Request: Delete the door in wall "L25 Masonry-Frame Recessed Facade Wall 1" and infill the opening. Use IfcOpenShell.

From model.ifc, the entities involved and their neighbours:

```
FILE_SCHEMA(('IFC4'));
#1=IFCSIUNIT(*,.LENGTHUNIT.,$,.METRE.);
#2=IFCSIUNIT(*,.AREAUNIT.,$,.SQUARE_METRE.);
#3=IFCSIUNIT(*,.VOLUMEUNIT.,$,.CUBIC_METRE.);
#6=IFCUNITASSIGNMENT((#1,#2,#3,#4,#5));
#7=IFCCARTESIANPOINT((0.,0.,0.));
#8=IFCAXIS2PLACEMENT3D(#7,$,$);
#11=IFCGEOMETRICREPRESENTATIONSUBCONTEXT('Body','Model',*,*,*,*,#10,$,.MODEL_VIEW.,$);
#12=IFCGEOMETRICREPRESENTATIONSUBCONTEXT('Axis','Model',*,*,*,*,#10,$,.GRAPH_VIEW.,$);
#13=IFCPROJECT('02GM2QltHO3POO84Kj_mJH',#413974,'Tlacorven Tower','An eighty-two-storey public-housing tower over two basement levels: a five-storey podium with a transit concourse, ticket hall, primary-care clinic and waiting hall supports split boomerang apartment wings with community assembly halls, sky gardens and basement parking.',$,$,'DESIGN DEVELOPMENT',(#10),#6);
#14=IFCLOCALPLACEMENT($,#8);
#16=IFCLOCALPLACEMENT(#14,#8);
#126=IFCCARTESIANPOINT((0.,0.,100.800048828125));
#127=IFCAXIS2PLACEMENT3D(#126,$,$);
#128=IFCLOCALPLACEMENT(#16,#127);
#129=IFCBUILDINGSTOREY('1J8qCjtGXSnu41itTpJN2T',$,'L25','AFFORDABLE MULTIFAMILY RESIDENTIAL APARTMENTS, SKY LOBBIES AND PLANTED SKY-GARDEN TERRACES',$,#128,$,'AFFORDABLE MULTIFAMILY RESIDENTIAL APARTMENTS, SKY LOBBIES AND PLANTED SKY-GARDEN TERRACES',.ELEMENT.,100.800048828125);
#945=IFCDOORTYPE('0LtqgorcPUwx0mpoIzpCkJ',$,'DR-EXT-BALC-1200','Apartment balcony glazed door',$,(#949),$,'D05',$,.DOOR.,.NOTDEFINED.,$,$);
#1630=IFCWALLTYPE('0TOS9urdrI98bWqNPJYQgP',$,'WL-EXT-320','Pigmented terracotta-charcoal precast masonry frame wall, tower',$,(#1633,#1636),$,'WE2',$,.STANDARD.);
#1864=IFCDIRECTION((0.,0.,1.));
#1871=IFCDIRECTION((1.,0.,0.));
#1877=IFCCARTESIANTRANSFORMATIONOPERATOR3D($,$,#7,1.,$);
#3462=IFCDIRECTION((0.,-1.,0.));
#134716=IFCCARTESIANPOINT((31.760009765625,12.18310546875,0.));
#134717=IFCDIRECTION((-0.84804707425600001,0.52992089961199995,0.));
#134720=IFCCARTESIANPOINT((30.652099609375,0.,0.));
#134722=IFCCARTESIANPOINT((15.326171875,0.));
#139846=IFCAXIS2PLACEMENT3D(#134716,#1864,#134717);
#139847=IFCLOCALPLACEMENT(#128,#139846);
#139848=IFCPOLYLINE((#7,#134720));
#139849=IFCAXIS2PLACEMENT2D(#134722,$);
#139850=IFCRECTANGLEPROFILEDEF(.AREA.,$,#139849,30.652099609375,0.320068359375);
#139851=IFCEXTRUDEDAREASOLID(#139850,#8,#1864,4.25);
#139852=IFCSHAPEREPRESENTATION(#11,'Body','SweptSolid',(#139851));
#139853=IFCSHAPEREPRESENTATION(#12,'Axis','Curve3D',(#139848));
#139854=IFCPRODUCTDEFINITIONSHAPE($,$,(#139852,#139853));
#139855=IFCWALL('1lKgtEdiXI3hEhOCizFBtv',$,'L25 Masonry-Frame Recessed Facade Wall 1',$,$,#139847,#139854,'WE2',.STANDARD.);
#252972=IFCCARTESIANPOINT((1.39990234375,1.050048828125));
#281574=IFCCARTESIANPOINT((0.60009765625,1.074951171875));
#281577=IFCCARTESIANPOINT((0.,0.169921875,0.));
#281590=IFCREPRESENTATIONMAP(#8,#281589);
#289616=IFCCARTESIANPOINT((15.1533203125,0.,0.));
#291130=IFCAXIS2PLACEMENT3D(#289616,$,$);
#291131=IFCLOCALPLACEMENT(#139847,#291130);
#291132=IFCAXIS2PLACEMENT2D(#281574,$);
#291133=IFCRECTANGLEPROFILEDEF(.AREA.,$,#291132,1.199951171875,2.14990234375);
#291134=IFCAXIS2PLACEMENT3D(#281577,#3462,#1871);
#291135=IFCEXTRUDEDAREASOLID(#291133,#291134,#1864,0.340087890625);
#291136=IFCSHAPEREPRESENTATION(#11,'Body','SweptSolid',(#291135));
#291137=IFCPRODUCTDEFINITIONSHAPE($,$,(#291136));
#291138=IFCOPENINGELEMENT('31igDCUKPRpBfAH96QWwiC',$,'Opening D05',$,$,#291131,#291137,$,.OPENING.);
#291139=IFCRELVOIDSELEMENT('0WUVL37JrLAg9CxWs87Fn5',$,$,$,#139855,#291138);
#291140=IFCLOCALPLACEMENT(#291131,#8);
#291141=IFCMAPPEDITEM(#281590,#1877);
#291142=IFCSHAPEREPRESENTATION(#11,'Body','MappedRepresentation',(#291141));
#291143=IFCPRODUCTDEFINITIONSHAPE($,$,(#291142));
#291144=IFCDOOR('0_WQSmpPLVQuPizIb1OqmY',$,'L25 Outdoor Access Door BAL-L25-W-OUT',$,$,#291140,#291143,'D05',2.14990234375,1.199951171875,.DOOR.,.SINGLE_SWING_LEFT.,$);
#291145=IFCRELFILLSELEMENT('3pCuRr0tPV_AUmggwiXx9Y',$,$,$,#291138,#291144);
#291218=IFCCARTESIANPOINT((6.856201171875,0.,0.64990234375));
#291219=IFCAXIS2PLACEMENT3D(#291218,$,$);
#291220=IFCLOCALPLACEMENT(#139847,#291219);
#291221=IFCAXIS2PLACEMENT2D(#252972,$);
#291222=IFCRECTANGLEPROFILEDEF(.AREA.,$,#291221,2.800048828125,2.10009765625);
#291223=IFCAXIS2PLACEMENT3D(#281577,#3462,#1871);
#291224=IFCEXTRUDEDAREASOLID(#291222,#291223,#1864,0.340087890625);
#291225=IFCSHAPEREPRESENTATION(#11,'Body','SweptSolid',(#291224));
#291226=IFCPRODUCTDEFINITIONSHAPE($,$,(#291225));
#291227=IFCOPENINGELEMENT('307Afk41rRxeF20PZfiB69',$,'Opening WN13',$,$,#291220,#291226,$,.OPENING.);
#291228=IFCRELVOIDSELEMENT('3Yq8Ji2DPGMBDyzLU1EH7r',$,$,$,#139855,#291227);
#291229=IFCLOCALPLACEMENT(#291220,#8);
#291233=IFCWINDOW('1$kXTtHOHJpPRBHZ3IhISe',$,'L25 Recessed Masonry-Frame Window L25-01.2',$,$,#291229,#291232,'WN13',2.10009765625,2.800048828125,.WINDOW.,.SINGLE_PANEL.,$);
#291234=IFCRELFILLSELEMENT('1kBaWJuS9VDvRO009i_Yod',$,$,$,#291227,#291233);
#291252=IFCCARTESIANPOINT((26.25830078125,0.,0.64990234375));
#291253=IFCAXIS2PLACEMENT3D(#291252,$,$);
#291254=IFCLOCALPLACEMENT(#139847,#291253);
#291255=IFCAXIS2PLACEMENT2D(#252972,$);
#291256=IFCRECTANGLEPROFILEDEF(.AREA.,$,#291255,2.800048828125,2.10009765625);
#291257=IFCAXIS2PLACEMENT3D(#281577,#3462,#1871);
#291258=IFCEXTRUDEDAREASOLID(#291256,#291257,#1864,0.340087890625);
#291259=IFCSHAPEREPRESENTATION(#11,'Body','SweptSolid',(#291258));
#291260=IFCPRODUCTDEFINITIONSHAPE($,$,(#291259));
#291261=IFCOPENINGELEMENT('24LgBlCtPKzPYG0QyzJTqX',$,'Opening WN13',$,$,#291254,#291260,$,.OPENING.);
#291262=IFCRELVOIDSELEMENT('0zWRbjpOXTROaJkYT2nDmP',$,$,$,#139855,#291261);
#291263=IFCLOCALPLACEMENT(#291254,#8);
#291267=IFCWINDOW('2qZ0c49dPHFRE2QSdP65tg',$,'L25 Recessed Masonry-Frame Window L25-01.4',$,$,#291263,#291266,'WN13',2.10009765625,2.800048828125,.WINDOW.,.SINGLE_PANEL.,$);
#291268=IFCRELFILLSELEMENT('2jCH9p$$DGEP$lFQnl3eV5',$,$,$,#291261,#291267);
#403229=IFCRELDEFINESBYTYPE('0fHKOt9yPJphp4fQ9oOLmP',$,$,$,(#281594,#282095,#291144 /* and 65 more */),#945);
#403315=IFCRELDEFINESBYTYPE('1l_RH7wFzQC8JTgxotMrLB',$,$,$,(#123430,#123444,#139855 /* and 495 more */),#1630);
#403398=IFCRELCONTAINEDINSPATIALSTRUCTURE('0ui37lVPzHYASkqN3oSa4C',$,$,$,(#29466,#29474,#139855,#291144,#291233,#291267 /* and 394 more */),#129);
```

```python
import ifcopenshell
import ifcopenshell.api.feature
import ifcopenshell.api.root
import ifcopenshell.geom
import ifcopenshell.util.shape

model = ifcopenshell.open("model.ifc")
settings = ifcopenshell.geom.settings()


def volume(element):
    """Net volume in cubic metres, openings subtracted."""
    shape = ifcopenshell.geom.create_shape(settings, element)
    return ifcopenshell.util.shape.get_volume(shape.geometry)


door = model.by_id(291144)
opening = door.FillsVoids[0].RelatingOpeningElement
wall = opening.VoidsElements[0].RelatingBuildingElement
before = volume(wall)

ifcopenshell.api.root.remove_product(model, product=door)
ifcopenshell.api.feature.remove_feature(model, feature=opening)

after = volume(wall)

print(f"wall volume {before:.3f} -> {after:.3f} m3")

model.write("model_edited.ifc")
```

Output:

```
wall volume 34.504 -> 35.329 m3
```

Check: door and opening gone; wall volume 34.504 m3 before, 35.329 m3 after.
